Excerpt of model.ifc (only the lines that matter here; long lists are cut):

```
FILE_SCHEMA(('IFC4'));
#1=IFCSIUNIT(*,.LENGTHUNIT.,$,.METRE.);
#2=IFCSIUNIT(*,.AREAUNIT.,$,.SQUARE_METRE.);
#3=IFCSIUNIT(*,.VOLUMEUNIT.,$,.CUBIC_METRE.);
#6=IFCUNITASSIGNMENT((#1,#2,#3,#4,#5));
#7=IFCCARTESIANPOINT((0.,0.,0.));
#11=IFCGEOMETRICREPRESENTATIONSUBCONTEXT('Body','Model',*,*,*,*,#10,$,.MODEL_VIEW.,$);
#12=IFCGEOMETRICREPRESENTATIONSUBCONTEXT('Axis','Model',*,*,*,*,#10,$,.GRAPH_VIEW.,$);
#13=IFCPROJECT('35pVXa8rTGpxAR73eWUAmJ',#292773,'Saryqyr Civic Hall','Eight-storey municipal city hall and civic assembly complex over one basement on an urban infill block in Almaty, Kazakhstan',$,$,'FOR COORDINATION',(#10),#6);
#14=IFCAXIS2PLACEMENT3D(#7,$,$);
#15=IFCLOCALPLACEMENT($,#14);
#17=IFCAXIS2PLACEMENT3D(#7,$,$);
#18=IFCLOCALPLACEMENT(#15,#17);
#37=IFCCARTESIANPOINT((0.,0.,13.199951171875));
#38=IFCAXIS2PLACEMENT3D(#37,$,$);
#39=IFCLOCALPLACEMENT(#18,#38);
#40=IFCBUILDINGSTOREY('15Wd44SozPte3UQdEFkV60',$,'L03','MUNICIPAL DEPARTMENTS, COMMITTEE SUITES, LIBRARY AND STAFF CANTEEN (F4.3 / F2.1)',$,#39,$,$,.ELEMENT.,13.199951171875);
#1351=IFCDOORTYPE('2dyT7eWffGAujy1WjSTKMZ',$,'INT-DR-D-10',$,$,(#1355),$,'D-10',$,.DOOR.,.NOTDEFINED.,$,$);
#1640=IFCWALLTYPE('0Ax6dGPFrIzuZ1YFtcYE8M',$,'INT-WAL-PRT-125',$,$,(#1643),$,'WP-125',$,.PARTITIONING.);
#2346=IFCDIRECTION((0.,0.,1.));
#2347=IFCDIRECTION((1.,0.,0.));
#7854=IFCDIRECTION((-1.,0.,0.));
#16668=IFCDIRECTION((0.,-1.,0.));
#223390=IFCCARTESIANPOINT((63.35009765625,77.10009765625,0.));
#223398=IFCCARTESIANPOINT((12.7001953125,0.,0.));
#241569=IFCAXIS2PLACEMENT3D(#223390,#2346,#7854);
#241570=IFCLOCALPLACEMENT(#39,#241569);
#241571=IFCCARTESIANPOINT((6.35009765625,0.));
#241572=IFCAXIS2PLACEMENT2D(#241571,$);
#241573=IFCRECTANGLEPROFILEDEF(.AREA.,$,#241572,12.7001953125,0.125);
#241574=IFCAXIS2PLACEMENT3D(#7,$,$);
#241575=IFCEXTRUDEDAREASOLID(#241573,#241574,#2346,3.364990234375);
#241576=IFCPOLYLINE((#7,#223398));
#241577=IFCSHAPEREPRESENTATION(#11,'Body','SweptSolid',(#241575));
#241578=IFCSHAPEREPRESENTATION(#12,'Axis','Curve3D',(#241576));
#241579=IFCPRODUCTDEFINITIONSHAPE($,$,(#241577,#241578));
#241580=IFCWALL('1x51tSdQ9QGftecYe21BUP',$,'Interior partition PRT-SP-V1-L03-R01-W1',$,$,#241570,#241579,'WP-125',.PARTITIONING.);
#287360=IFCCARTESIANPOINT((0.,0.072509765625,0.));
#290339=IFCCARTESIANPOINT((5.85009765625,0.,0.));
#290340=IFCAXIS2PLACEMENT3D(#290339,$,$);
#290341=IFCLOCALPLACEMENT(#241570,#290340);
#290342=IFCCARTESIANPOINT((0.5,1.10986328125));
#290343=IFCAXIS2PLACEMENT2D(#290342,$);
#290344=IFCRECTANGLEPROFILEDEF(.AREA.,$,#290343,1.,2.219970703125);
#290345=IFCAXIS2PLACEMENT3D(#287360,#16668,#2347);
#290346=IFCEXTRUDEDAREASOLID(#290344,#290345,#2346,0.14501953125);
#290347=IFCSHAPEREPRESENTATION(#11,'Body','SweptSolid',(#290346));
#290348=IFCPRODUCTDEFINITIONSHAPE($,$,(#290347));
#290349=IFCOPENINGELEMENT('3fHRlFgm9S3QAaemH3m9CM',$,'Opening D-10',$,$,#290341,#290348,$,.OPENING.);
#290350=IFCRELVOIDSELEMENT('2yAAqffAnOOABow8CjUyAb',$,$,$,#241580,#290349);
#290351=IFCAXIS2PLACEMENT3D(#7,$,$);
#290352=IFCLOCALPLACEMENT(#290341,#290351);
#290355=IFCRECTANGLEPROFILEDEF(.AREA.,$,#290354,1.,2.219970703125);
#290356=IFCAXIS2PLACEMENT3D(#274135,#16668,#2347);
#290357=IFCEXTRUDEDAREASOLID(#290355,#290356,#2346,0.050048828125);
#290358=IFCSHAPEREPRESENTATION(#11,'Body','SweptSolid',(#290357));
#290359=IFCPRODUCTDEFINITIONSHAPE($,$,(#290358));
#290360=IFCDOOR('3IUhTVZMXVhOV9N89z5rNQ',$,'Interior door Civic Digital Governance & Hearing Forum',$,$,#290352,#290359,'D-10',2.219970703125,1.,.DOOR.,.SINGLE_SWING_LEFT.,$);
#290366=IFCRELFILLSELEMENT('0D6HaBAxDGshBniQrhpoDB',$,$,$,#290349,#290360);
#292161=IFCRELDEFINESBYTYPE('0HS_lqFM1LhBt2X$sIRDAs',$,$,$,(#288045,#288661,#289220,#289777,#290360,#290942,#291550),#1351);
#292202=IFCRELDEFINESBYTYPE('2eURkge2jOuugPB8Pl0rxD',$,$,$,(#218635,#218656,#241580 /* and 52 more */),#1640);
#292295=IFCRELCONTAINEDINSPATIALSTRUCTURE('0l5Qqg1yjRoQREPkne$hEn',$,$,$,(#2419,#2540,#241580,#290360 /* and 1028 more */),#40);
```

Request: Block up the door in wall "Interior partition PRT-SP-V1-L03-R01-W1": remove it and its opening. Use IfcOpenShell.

```python
import ifcopenshell
import ifcopenshell.api.feature
import ifcopenshell.api.root
import ifcopenshell.geom
import ifcopenshell.util.shape

model = ifcopenshell.open("model.ifc")
settings = ifcopenshell.geom.settings()


def volume(element):
    """Net volume in cubic metres, openings subtracted."""
    shape = ifcopenshell.geom.create_shape(settings, element)
    return ifcopenshell.util.shape.get_volume(shape.geometry)


door = model.by_guid("3IUhTVZMXVhOV9N89z5rNQ")
opening = door.FillsVoids[0].RelatingOpeningElement
wall = opening.VoidsElements[0].RelatingBuildingElement
before = volume(wall)

ifcopenshell.api.root.remove_product(model, product=door)
ifcopenshell.api.feature.remove_feature(model, feature=opening)

after = volume(wall)

print(f"wall volume {before:.3f} -> {after:.3f} m3")

model.write("model_edited.ifc")
```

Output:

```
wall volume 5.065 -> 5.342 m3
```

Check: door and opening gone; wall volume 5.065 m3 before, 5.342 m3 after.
